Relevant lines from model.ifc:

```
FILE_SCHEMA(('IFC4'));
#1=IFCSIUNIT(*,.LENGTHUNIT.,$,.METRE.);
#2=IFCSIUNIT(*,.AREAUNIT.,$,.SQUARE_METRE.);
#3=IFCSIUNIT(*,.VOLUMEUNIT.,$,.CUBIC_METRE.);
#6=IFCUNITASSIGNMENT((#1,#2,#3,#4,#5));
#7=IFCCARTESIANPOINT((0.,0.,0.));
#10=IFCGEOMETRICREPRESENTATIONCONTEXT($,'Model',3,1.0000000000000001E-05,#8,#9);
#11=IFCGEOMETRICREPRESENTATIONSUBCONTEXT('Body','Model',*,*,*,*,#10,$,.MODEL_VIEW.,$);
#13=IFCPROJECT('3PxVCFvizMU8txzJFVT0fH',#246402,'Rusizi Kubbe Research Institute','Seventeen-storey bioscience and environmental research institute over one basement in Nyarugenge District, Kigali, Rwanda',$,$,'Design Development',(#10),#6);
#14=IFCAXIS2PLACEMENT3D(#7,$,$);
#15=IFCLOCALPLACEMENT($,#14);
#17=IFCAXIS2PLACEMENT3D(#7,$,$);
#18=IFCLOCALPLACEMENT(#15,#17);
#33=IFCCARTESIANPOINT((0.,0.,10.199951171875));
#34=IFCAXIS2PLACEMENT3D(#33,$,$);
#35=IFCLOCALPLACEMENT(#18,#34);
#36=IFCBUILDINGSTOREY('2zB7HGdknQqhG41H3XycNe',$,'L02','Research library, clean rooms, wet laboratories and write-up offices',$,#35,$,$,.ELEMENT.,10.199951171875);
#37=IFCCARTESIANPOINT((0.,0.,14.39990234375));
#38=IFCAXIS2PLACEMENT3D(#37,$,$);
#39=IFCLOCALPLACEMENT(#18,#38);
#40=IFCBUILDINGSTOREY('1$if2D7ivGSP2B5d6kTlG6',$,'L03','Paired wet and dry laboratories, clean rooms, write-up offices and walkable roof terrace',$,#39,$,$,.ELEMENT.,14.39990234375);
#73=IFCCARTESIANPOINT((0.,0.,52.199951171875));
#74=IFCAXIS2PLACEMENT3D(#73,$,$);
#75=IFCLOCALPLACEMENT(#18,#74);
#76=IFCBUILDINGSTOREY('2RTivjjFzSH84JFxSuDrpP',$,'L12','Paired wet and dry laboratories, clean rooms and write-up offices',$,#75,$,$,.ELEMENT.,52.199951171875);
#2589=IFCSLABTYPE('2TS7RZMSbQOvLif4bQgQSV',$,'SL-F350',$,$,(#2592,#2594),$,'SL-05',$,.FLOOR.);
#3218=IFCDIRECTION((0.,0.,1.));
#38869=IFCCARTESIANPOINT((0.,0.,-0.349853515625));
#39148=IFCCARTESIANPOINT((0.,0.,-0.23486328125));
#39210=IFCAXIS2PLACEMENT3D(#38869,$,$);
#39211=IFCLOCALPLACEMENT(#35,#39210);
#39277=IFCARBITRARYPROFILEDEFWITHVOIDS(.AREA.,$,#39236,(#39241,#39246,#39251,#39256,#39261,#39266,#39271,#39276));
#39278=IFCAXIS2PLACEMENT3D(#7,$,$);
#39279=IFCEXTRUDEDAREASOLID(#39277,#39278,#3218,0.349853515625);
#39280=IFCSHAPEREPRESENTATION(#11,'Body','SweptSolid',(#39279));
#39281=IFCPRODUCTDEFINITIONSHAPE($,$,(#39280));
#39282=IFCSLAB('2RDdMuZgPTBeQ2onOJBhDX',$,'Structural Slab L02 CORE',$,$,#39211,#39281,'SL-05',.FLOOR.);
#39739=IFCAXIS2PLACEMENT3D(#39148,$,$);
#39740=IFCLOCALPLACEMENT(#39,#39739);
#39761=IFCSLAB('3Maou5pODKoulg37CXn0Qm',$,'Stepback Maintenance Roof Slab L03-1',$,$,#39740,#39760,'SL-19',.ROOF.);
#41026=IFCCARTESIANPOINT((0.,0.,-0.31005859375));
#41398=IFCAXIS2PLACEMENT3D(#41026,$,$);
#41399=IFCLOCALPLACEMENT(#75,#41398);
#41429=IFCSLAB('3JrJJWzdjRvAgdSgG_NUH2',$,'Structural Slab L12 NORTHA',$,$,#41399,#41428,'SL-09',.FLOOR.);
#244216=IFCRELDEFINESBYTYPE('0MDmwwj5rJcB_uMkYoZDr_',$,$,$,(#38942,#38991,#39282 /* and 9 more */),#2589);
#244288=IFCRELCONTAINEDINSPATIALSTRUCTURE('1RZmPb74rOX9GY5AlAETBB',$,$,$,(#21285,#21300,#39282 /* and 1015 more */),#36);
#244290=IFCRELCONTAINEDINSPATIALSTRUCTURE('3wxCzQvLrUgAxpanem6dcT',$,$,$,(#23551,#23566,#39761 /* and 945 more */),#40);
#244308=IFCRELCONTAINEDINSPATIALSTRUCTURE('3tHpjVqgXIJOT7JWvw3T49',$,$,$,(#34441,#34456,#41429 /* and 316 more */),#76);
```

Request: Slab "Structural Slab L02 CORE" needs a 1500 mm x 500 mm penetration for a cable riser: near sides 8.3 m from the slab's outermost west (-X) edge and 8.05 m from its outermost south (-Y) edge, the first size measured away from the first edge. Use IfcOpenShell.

```python
import numpy as np
import ifcopenshell
import ifcopenshell.api.feature
import ifcopenshell.api.geometry
import ifcopenshell.api.root
import ifcopenshell.geom
import ifcopenshell.util.placement
import ifcopenshell.util.representation
import ifcopenshell.util.shape
import ifcopenshell.util.unit

model = ifcopenshell.open("model.ifc")
unit_scale = ifcopenshell.util.unit.calculate_unit_scale(model)
settings = ifcopenshell.geom.settings()


def volume(element):
    """Net volume in cubic metres, openings subtracted."""
    shape = ifcopenshell.geom.create_shape(settings, element)
    return ifcopenshell.util.shape.get_volume(shape.geometry)


slab = model.by_guid("2RDdMuZgPTBeQ2onOJBhDX")
before = volume(slab)

# Extent in the slab's own axes, in metres. The edges named are its -X and -Y sides.
slab_shape = ifcopenshell.geom.create_shape(settings, slab)
vertices = ifcopenshell.util.shape.get_vertices(slab_shape.geometry)
x_min, y_min, bottom = vertices.min(axis=0)
top = vertices[:, 2].max()

opening = ifcopenshell.api.root.create_entity(model, ifc_class="IfcOpeningElement", name="Cable riser opening", predefined_type="OPENING")
context = ifcopenshell.util.representation.get_context(model, "Model", "Body", "MODEL_VIEW")
width, depth = 1.5, 0.5
outline = [(0.0, 0.0), (width, 0.0), (width, depth), (0.0, depth), (0.0, 0.0)]
# Overshoot both faces by 50 mm so the cut is clean.
shape = ifcopenshell.api.geometry.add_slab_representation(
    model, context=context, depth=top - bottom + 0.1, polyline=outline
)
ifcopenshell.api.geometry.assign_representation(model, product=opening, representation=shape)

matrix = ifcopenshell.util.placement.get_local_placement(slab.ObjectPlacement)
matrix[:, 3] = matrix @ np.append(np.array([x_min + 8.3, y_min + 8.05, bottom - 0.05]) / unit_scale, 1.0)
ifcopenshell.api.geometry.edit_object_placement(model, product=opening, matrix=matrix, is_si=False)
ifcopenshell.api.feature.add_feature(model, feature=opening, element=slab)

after = volume(slab)

print(f"slab volume {before:.3f} -> {after:.3f} m3")

model.write("model_edited.ifc")
```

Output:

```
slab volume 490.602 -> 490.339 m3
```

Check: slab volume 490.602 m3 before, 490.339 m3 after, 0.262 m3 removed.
